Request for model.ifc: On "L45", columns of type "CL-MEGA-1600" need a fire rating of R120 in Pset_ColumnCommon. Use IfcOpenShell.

First a look at what the model holds.

```python
import ifcopenshell
import ifcopenshell.util.element

model = ifcopenshell.open("model.ifc")
print(model.schema)
storey = next(s for s in model.by_type("IfcBuildingStorey") if s.Name == "L45")
columns = [e for e in ifcopenshell.util.element.get_decomposition(storey) if e.is_a("IfcColumn")]
seen = {}
for e in columns:
    element_type = ifcopenshell.util.element.get_type(e)
    key = (element_type.Name if element_type != e and element_type else None, ifcopenshell.util.element.get_pset(e, "Pset_ColumnCommon", "FireRating"))
    seen[key] = seen.get(key, 0) + 1
for (name, value), count in sorted(seen.items(), key=str):
    print(count, "x", name, "|", value)
```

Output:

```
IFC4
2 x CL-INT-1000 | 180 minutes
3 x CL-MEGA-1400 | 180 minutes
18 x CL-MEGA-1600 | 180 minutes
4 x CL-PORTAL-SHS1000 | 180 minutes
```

```python
import ifcopenshell
import ifcopenshell.api.pset
import ifcopenshell.util.element

model = ifcopenshell.open("model.ifc")

storey = next(s for s in model.by_type("IfcBuildingStorey") if s.Name == "L45")
columns = [e for e in ifcopenshell.util.element.get_decomposition(storey) if e.is_a("IfcColumn")]

count = 0
for e in columns:
    element_type = ifcopenshell.util.element.get_type(e)
    if element_type in (None, e) or element_type.Name != "CL-MEGA-1600":
        continue
    found = ifcopenshell.util.element.get_pset(e, "Pset_ColumnCommon", should_inherit=False)
    if found:
        pset = model.by_id(found["id"])
        if len(ifcopenshell.util.element.get_elements_by_pset(pset)) > 1:
            pset = ifcopenshell.api.pset.unshare_pset(model, products=[e], pset=pset)[0]
    else:
        pset = ifcopenshell.api.pset.add_pset(model, product=e, name="Pset_ColumnCommon")
    ifcopenshell.api.pset.edit_pset(model, pset=pset, properties={"FireRating": "R120"})
    count += 1

print(count, "columns updated")

model.write("model_rev.ifc")
```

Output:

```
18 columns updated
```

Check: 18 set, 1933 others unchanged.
